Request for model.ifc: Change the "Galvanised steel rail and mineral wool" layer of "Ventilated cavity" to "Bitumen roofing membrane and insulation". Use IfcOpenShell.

First a look at what the model holds.

```python
import ifcopenshell
import ifcopenshell.util.element

model = ifcopenshell.open("model.ifc")
print(model.schema)
for layer_set in model.by_type("IfcMaterialLayerSet"):
    if layer_set.LayerSetName == "Ventilated cavity":
        for layer in layer_set.MaterialLayers:
            print(layer.id(), layer.Material and layer.Material.Name, layer.LayerThickness, sep=" | ")
        print(len(ifcopenshell.util.element.get_elements_by_material(model, layer_set)), "elements and types use it")
print(sorted(m.Name for m in model.by_type("IfcMaterial") if m.Name)[:60])
```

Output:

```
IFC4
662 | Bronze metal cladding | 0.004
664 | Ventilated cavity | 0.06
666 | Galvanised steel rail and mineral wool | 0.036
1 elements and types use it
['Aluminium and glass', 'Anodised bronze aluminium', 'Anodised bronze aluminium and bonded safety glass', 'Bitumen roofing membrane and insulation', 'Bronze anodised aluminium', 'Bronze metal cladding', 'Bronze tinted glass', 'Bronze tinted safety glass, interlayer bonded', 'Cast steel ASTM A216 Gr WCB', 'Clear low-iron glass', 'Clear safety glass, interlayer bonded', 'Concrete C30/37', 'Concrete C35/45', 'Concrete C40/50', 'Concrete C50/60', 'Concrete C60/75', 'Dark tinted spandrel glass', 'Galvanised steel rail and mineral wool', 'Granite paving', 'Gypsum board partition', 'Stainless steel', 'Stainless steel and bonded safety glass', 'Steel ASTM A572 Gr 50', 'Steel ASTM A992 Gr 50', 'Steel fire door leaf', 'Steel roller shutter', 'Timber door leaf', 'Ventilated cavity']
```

```python
import ifcopenshell
import ifcopenshell.api.material

model = ifcopenshell.open("model.ifc")

layer_set = next(s for s in model.by_type("IfcMaterialLayerSet") if s.LayerSetName == "Ventilated cavity")
layer = next(l for l in layer_set.MaterialLayers if l.Material and l.Material.Name == "Galvanised steel rail and mineral wool")
material = next(m for m in model.by_type("IfcMaterial") if m.Name == "Bitumen roofing membrane and insulation")

# Point this one layer at the other material; renaming the old one would change it everywhere.
ifcopenshell.api.material.edit_layer(model, layer=layer, attributes={}, material=material)

print([l.Material.Name if l.Material else None for l in layer_set.MaterialLayers])

model.write("model_updated.ifc")
```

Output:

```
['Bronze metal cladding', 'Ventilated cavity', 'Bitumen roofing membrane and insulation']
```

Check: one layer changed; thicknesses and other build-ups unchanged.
